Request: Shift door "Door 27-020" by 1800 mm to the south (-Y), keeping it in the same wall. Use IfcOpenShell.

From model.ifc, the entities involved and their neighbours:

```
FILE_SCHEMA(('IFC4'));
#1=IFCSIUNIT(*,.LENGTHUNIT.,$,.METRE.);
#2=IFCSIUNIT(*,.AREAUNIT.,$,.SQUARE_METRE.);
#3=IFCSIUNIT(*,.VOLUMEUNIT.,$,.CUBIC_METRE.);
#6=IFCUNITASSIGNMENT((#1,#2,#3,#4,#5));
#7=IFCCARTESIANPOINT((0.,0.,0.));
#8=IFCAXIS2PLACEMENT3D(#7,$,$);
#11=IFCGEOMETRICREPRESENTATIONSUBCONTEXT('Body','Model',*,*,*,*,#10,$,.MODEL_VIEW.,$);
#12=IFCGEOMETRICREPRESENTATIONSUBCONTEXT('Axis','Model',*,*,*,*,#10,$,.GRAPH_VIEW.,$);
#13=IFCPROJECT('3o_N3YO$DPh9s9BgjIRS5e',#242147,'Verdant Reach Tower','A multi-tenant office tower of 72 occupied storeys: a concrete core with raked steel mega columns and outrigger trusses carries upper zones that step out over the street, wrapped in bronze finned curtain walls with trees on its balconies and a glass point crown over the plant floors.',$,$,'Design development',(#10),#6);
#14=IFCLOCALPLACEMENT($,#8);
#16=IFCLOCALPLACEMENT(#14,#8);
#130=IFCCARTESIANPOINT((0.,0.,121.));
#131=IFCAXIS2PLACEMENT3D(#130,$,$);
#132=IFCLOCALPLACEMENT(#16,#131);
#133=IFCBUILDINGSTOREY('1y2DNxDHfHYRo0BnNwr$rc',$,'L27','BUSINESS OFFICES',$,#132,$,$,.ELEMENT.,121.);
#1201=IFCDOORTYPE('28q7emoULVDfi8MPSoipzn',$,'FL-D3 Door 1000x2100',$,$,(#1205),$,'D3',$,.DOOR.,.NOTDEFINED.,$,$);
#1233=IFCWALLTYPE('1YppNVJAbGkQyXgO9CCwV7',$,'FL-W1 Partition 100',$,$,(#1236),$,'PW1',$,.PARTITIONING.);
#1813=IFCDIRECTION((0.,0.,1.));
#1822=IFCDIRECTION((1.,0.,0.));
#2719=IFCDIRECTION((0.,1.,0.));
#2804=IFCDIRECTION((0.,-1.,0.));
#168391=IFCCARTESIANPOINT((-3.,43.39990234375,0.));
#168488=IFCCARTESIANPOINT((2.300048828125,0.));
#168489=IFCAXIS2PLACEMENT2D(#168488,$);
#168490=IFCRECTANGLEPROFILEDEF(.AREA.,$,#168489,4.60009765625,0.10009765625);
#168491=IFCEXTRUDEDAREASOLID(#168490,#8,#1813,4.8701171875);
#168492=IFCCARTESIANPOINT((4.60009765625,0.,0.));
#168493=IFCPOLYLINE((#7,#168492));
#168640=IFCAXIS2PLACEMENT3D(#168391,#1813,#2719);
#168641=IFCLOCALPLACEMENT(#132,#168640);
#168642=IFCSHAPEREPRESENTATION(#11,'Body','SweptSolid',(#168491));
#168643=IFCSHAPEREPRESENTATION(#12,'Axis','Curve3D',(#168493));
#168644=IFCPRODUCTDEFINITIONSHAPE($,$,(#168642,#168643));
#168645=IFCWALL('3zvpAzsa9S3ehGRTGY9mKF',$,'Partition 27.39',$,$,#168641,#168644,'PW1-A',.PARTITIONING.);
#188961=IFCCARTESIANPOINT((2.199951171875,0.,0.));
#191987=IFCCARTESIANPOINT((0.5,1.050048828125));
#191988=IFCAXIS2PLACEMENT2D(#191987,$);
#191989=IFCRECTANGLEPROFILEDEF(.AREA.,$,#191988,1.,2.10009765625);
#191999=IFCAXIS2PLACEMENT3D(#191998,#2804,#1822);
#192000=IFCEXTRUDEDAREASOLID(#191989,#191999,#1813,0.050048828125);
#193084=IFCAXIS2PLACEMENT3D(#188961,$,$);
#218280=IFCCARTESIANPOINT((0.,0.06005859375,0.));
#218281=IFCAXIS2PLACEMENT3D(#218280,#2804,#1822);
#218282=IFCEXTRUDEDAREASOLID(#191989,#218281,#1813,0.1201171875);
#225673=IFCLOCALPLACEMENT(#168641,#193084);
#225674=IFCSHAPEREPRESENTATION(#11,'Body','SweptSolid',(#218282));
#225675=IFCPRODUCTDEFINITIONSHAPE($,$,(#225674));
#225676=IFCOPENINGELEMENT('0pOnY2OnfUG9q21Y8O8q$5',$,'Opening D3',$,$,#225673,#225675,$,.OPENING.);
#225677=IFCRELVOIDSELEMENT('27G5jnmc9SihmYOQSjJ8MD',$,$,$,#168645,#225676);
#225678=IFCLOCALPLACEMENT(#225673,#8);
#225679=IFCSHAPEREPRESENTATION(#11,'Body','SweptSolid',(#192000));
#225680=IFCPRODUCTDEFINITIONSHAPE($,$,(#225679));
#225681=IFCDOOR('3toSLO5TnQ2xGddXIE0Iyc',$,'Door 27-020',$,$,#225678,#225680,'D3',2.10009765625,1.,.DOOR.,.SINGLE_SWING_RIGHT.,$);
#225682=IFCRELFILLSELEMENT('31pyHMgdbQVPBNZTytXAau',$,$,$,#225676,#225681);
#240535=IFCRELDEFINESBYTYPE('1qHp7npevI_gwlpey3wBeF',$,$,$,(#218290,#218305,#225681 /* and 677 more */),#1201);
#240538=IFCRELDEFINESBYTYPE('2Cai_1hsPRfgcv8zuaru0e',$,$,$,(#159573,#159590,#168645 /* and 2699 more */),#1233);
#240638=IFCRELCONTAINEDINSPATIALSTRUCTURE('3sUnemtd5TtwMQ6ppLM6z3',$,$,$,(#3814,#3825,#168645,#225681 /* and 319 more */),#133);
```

```python
import ifcopenshell
import ifcopenshell.api.geometry
import ifcopenshell.util.placement
import ifcopenshell.util.unit

model = ifcopenshell.open("model.ifc")
unit_scale = ifcopenshell.util.unit.calculate_unit_scale(model)

door = model.by_id(225681)
opening = door.FillsVoids[0].RelatingOpeningElement
wall = opening.VoidsElements[0].RelatingBuildingElement

wall_matrix = ifcopenshell.util.placement.get_local_placement(wall.ObjectPlacement)
shift = wall_matrix[:3, 0] * -1.8 / unit_scale
before = ifcopenshell.util.placement.get_local_placement(door.ObjectPlacement)[:3, 3].copy()

# The door is placed relative to its opening, so it follows when the opening moves.
matrix = ifcopenshell.util.placement.get_local_placement(opening.ObjectPlacement)
matrix[:3, 3] += shift
ifcopenshell.api.geometry.edit_object_placement(
    model, product=opening, matrix=matrix, is_si=False, should_transform_children=True
)

after = ifcopenshell.util.placement.get_local_placement(door.ObjectPlacement)[:3, 3]
print("door moved by", (after - before).round(3) + 0.0)

model.write("model_edited.ifc")
```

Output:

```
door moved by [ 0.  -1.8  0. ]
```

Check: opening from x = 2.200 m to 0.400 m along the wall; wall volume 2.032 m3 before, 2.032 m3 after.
